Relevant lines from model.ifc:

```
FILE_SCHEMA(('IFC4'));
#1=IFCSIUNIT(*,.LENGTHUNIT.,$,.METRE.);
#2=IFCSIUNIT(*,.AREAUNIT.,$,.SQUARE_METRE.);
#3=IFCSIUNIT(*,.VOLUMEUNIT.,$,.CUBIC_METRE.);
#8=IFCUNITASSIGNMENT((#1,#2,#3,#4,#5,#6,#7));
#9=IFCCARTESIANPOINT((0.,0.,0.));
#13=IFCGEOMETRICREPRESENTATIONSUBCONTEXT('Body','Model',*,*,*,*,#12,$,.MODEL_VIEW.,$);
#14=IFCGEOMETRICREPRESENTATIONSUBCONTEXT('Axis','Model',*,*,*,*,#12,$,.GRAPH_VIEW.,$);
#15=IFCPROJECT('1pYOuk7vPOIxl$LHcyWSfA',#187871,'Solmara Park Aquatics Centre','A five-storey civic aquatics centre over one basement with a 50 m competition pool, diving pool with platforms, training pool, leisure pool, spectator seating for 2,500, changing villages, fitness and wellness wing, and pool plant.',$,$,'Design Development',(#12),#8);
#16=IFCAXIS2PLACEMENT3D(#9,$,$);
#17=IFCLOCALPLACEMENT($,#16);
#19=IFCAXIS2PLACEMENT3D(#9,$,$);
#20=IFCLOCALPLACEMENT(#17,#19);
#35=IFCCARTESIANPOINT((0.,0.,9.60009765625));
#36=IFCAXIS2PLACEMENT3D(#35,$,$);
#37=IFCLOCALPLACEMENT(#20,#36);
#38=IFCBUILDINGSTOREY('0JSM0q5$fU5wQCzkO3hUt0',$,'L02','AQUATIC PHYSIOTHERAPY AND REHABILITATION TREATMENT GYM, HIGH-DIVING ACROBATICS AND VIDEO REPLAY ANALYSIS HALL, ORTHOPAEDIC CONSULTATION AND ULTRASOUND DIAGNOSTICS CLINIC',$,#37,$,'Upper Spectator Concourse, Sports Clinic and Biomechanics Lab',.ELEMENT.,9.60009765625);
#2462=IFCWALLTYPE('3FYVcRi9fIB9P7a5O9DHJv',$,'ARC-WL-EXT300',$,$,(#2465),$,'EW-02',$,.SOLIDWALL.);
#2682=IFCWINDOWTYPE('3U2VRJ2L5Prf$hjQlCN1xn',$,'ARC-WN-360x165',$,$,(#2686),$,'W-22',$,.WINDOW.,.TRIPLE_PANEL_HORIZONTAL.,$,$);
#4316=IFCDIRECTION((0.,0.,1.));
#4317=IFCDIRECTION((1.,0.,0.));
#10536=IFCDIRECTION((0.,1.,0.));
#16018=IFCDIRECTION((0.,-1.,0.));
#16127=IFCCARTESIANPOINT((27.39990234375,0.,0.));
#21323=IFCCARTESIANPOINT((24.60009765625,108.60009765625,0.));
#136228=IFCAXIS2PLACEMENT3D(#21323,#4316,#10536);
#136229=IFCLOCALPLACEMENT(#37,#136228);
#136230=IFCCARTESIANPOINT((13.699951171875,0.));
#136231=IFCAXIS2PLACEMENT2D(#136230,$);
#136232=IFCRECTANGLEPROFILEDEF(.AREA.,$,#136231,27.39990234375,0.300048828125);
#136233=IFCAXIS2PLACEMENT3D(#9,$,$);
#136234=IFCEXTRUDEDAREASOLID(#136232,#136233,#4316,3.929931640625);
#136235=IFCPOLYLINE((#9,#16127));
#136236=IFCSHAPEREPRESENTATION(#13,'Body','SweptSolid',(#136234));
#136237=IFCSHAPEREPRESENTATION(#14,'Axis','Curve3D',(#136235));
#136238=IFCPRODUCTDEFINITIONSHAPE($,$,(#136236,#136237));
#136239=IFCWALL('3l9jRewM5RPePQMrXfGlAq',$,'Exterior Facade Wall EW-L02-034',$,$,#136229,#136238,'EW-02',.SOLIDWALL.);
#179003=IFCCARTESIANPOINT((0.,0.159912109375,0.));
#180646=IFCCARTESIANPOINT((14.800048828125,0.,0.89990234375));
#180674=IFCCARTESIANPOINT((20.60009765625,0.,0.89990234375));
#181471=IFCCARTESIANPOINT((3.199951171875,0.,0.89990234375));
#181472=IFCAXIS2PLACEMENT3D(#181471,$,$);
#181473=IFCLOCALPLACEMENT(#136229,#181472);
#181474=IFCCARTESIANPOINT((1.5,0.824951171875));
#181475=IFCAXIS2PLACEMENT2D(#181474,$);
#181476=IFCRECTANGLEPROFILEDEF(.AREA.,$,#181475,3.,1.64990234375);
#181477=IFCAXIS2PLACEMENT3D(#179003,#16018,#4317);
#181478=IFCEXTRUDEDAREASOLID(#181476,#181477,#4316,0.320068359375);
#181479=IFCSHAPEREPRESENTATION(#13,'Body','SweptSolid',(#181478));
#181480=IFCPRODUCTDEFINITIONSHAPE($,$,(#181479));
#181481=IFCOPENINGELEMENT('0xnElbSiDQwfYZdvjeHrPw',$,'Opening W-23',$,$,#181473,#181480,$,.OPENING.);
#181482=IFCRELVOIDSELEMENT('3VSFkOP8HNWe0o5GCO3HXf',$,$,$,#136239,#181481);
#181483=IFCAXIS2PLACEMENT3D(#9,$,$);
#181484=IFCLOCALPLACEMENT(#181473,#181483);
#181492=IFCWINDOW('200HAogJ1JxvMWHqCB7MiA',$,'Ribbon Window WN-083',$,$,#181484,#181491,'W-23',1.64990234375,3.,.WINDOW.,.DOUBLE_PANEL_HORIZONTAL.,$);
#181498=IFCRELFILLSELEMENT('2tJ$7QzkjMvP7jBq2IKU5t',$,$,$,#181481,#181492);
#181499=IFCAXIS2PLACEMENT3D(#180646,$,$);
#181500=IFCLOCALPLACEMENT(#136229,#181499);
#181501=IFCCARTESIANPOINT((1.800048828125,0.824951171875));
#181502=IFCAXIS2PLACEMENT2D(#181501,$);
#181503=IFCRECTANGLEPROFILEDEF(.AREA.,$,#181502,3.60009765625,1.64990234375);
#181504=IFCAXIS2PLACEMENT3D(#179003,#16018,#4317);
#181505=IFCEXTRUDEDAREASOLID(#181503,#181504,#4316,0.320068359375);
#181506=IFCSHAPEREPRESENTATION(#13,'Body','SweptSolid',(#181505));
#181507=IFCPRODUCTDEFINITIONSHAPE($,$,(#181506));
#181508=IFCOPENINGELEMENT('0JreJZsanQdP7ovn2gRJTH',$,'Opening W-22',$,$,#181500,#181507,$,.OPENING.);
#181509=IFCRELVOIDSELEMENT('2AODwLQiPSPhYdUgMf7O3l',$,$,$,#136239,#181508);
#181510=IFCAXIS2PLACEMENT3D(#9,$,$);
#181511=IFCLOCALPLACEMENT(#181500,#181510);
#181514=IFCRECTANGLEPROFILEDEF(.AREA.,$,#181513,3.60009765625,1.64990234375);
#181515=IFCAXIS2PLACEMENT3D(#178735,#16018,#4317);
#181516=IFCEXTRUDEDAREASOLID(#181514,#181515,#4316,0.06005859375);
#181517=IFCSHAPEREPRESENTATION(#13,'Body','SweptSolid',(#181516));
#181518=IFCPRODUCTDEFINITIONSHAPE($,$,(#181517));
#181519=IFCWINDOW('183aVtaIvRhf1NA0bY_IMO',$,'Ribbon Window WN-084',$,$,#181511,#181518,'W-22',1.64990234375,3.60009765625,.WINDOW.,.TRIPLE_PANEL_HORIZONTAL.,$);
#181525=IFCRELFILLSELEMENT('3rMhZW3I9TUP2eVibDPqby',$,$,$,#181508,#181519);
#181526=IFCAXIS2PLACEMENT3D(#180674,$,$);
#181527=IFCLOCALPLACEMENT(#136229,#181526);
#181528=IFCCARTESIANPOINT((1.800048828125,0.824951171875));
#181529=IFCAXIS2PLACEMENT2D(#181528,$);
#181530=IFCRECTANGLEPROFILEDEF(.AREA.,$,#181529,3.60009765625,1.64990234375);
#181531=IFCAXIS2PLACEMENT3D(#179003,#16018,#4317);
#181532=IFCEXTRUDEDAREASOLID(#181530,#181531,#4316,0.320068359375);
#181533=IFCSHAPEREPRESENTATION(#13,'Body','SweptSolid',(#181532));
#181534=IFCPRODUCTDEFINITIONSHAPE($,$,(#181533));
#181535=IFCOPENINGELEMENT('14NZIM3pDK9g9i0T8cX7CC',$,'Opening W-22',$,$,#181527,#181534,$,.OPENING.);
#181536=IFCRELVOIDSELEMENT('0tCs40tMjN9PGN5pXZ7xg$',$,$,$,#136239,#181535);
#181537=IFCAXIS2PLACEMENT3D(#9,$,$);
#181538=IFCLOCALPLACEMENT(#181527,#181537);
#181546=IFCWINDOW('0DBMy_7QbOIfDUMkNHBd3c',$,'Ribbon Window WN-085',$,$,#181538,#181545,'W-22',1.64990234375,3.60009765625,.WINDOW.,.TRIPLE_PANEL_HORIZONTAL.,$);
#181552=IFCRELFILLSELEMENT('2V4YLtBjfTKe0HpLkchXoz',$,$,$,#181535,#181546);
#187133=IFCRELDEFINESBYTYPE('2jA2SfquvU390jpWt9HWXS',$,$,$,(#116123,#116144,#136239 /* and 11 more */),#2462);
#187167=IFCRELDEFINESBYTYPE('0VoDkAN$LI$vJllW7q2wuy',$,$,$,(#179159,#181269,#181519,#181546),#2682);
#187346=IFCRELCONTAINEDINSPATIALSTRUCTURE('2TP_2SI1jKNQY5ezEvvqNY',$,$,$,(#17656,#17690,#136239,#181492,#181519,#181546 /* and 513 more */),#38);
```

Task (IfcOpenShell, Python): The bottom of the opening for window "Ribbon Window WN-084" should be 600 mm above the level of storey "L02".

```python
import numpy as np
import ifcopenshell
import ifcopenshell.api.geometry
import ifcopenshell.geom
import ifcopenshell.util.element
import ifcopenshell.util.placement
import ifcopenshell.util.shape
import ifcopenshell.util.unit

model = ifcopenshell.open("model.ifc")
unit_scale = ifcopenshell.util.unit.calculate_unit_scale(model)

window = model.by_guid("183aVtaIvRhf1NA0bY_IMO")
opening = window.FillsVoids[0].RelatingOpeningElement
storey = ifcopenshell.util.element.get_container(window, ifc_class="IfcBuildingStorey")
level = ifcopenshell.util.placement.get_local_placement(storey.ObjectPlacement)[2, 3]

# The opening's origin need not be at the sill, so measure its lowest point.
shape = ifcopenshell.geom.create_shape(ifcopenshell.geom.settings(), opening)
bottom = ifcopenshell.util.shape.get_shape_bottom_elevation(shape, shape.geometry) / unit_scale
dz = level + 0.6 / unit_scale - bottom

shift = np.array([0.0, 0.0, dz])
# The window is placed relative to its opening, so it follows when the opening moves.
matrix = ifcopenshell.util.placement.get_local_placement(opening.ObjectPlacement)
matrix[:3, 3] += shift
ifcopenshell.api.geometry.edit_object_placement(
    model, product=opening, matrix=matrix, is_si=False, should_transform_children=True
)

print(f"moved by {dz * unit_scale:+.3f} m")

model.write("model_v2.ifc")
```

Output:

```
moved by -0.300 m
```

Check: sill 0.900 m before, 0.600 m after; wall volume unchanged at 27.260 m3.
